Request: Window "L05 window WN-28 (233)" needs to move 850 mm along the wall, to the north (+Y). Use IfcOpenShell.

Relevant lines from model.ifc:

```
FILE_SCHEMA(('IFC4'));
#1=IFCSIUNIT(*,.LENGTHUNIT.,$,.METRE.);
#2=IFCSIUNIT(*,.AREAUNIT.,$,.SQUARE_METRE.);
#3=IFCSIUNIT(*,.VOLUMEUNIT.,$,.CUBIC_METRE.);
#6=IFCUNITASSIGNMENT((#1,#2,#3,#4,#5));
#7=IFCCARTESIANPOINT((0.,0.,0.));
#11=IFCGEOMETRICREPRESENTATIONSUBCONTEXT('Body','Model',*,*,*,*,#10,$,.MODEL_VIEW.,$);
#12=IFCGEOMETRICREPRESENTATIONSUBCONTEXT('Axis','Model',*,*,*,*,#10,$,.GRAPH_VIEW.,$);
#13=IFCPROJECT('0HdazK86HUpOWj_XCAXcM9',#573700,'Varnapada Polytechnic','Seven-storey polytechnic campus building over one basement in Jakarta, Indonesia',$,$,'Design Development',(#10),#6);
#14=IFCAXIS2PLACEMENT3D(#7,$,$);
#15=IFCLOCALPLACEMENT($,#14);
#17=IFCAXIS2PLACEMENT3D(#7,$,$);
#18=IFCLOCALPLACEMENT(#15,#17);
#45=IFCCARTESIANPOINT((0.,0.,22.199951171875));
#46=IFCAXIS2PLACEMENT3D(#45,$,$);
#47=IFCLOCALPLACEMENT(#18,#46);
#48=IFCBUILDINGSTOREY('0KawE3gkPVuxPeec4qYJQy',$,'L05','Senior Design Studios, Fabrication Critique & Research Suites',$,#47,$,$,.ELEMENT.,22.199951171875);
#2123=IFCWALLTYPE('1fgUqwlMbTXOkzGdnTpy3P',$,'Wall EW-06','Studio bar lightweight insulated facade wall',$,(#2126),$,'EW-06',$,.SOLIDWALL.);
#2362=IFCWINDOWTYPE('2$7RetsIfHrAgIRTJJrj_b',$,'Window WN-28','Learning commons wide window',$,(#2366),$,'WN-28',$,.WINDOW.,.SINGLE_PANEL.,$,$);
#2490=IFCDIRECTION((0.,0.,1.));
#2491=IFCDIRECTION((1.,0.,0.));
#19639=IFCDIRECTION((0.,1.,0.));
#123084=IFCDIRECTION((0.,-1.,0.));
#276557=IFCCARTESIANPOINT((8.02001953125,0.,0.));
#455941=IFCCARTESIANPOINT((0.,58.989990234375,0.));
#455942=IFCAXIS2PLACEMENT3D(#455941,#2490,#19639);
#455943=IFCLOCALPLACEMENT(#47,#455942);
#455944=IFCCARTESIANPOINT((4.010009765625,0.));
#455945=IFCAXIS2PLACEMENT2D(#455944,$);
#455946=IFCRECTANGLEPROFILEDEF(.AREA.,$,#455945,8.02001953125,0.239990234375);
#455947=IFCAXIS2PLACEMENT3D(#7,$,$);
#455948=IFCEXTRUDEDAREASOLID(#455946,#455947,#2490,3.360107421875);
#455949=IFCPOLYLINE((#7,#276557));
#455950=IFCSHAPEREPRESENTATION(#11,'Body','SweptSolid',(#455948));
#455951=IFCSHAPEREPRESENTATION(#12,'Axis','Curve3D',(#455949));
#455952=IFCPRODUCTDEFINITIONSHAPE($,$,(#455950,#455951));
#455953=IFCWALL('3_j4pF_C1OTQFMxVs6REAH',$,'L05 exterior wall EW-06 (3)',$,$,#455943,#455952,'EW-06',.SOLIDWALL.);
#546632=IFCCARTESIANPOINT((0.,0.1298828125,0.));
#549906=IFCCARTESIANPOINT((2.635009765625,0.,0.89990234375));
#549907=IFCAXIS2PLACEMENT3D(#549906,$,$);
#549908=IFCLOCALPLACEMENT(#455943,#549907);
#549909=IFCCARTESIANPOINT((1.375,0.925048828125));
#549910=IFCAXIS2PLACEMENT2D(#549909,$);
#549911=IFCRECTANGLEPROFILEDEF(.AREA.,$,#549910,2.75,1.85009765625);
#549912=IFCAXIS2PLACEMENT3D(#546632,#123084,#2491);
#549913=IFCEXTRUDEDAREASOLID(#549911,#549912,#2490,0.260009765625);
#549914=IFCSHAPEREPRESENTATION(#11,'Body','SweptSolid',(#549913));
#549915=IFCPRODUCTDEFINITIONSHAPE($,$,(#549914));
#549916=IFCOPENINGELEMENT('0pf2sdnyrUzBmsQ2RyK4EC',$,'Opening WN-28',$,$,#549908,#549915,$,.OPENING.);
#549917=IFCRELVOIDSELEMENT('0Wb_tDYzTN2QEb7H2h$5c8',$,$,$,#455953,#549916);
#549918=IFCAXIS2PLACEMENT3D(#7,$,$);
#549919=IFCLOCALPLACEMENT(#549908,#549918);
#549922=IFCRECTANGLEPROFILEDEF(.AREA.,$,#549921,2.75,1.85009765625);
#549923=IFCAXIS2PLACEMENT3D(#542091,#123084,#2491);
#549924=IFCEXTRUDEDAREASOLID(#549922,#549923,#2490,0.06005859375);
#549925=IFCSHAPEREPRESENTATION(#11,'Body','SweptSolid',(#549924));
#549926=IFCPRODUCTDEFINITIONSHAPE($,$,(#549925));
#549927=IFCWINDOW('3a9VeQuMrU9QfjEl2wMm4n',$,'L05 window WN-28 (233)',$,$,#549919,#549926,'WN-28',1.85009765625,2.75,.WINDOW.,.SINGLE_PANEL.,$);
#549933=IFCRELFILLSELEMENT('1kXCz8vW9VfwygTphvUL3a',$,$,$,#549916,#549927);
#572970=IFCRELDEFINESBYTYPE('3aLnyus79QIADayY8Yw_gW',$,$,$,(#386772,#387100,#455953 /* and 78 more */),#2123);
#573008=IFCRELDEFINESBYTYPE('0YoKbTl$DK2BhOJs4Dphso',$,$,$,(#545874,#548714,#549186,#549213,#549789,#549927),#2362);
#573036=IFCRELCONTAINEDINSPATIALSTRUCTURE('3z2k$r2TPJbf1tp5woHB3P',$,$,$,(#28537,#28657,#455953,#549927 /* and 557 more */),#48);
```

```python
import ifcopenshell
import ifcopenshell.api.geometry
import ifcopenshell.util.placement

model = ifcopenshell.open("model.ifc")

window = model.by_guid("3a9VeQuMrU9QfjEl2wMm4n")
opening = window.FillsVoids[0].RelatingOpeningElement
wall = opening.VoidsElements[0].RelatingBuildingElement

wall_matrix = ifcopenshell.util.placement.get_local_placement(wall.ObjectPlacement)
shift = wall_matrix[:3, 0] * 0.85
before = ifcopenshell.util.placement.get_local_placement(window.ObjectPlacement)[:3, 3].copy()

# The window is placed relative to its opening, so it follows when the opening moves.
matrix = ifcopenshell.util.placement.get_local_placement(opening.ObjectPlacement)
matrix[:3, 3] += shift
ifcopenshell.api.geometry.edit_object_placement(
    model, product=opening, matrix=matrix, is_si=False, should_transform_children=True
)

after = ifcopenshell.util.placement.get_local_placement(window.ObjectPlacement)[:3, 3]
print("window moved by", (after - before).round(3) + 0.0)

model.write("model_rev.ifc")
```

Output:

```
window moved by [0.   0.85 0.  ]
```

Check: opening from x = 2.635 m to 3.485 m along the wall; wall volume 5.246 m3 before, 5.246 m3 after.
